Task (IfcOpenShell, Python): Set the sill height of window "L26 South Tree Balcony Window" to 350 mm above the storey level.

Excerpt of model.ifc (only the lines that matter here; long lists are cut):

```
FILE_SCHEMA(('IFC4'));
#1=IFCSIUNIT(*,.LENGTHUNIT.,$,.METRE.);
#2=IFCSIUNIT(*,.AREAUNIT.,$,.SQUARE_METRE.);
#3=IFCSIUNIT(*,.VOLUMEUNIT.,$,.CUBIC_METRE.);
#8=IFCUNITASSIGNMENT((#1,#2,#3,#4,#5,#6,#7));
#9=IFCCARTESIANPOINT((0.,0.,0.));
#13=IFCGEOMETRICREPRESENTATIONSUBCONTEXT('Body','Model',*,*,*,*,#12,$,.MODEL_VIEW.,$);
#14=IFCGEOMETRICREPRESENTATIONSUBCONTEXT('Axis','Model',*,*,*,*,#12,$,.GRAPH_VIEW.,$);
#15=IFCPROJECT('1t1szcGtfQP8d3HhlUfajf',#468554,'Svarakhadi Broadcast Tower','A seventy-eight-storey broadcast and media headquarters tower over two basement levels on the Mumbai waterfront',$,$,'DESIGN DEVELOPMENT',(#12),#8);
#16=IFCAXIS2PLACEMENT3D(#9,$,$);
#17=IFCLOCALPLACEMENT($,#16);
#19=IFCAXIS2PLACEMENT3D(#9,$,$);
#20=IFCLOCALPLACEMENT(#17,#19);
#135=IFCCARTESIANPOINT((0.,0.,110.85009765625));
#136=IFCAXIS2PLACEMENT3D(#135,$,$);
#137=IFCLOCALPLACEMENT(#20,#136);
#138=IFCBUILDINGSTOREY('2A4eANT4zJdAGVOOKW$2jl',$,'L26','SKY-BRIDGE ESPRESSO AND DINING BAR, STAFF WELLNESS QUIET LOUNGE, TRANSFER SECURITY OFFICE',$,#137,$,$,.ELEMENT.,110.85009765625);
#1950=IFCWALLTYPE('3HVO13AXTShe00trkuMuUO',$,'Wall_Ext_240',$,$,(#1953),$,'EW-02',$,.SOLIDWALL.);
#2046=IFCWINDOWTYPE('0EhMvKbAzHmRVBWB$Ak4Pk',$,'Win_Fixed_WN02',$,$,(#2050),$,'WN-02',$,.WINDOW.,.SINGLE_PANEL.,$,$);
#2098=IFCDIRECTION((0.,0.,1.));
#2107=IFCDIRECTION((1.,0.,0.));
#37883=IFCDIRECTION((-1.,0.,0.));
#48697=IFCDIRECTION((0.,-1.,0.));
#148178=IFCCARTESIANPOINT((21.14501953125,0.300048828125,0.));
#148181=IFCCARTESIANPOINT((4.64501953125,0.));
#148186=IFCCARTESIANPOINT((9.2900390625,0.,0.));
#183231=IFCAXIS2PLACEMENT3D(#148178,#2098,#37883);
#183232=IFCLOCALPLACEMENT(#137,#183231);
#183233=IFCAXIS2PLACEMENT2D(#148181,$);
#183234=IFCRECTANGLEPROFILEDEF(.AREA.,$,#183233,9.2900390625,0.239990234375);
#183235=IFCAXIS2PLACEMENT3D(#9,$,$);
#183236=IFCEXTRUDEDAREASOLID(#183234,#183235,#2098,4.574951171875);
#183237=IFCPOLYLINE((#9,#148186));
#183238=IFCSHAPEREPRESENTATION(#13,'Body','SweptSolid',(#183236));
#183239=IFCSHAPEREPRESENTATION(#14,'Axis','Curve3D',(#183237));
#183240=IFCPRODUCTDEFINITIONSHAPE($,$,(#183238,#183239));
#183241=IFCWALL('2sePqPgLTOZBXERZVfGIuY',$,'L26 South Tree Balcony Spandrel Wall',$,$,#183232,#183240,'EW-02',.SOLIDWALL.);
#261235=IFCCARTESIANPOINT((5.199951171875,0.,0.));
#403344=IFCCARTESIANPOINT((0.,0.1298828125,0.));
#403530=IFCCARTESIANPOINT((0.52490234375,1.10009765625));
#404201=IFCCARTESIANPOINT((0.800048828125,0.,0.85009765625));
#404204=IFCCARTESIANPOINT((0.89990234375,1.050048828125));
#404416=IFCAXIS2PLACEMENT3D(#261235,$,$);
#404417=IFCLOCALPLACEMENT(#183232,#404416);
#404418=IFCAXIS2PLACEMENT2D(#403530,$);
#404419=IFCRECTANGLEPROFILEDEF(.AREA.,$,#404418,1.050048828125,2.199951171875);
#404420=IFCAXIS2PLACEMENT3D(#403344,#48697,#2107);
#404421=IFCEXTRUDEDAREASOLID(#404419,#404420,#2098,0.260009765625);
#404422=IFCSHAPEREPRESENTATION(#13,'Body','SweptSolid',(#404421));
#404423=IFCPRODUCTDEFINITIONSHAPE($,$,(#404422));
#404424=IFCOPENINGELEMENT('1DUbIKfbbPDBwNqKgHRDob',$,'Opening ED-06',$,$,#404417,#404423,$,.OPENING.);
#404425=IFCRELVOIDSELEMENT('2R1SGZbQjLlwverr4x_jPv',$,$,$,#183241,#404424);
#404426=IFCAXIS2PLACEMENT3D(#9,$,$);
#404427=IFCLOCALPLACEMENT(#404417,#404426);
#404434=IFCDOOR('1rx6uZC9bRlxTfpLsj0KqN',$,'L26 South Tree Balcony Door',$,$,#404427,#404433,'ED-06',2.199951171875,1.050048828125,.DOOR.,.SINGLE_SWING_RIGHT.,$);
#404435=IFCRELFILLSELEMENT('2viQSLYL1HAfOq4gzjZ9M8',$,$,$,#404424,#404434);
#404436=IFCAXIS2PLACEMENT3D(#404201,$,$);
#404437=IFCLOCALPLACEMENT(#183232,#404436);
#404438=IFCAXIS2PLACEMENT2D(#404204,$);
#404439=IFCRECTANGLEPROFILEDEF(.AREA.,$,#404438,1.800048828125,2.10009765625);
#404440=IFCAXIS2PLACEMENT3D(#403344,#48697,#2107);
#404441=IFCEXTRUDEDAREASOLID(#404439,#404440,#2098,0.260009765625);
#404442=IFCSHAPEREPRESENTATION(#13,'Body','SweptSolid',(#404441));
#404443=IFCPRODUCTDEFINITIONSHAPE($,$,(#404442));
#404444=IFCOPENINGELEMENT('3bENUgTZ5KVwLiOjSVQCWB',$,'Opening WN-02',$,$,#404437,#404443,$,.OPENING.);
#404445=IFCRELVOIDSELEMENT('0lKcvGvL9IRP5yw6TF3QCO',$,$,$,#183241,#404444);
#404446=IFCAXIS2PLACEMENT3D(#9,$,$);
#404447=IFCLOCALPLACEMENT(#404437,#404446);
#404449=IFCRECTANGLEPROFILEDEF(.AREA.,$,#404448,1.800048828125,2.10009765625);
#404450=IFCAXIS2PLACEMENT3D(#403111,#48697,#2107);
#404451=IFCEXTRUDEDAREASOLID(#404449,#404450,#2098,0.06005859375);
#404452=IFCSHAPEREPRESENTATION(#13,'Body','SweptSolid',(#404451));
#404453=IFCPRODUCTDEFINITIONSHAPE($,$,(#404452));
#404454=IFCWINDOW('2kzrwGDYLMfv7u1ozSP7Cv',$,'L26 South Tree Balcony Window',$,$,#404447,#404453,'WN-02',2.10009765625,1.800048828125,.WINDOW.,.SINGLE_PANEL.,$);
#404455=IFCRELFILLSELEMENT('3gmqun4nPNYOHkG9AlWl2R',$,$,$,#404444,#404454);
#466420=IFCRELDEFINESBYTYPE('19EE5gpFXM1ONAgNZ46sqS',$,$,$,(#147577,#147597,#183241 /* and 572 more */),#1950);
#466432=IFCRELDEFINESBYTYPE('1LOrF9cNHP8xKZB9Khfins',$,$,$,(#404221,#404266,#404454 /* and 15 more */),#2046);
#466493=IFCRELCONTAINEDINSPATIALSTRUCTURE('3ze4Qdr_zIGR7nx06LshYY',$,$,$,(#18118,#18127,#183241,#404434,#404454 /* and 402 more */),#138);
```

```python
import numpy as np
import ifcopenshell
import ifcopenshell.api.geometry
import ifcopenshell.geom
import ifcopenshell.util.element
import ifcopenshell.util.placement
import ifcopenshell.util.shape
import ifcopenshell.util.unit

model = ifcopenshell.open("model.ifc")
unit_scale = ifcopenshell.util.unit.calculate_unit_scale(model)

window = model.by_guid("2kzrwGDYLMfv7u1ozSP7Cv")
opening = window.FillsVoids[0].RelatingOpeningElement
storey = ifcopenshell.util.element.get_container(window, ifc_class="IfcBuildingStorey")
level = ifcopenshell.util.placement.get_local_placement(storey.ObjectPlacement)[2, 3]

# The opening's origin need not be at the sill, so measure its lowest point.
shape = ifcopenshell.geom.create_shape(ifcopenshell.geom.settings(), opening)
bottom = ifcopenshell.util.shape.get_shape_bottom_elevation(shape, shape.geometry) / unit_scale
dz = level + 0.35 - bottom

shift = np.array([0.0, 0.0, dz])
# The window is placed relative to its opening, so it follows when the opening moves.
matrix = ifcopenshell.util.placement.get_local_placement(opening.ObjectPlacement)
matrix[:3, 3] += shift
ifcopenshell.api.geometry.edit_object_placement(
    model, product=opening, matrix=matrix, is_si=False, should_transform_children=True
)

print(f"moved by {dz * unit_scale:+.3f} m")

model.write("model-out.ifc")
```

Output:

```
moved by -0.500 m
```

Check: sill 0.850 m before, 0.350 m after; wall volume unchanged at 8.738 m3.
